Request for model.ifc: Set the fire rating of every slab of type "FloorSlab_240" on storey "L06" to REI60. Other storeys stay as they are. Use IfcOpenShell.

First a look at what the model holds.

```python
import ifcopenshell
import ifcopenshell.util.element

model = ifcopenshell.open("model.ifc")
print(model.schema)
storey = next(s for s in model.by_type("IfcBuildingStorey") if s.Name == "L06")
slabs = [e for e in ifcopenshell.util.element.get_decomposition(storey) if e.is_a("IfcSlab")]
seen = {}
for e in slabs:
    element_type = ifcopenshell.util.element.get_type(e)
    key = (element_type.Name if element_type != e and element_type else None, ifcopenshell.util.element.get_pset(e, "Pset_SlabCommon", "FireRating"))
    seen[key] = seen.get(key, 0) + 1
for (name, value), count in sorted(seen.items(), key=str):
    print(count, "x", name, "|", value)
```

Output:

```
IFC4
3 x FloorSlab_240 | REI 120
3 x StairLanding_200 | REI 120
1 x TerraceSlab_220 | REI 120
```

```python
import ifcopenshell
import ifcopenshell.api.pset
import ifcopenshell.util.element

model = ifcopenshell.open("model.ifc")

storey = next(s for s in model.by_type("IfcBuildingStorey") if s.Name == "L06")
slabs = [e for e in ifcopenshell.util.element.get_decomposition(storey) if e.is_a("IfcSlab")]

count = 0
for e in slabs:
    element_type = ifcopenshell.util.element.get_type(e)
    if element_type in (None, e) or element_type.Name != "FloorSlab_240":
        continue
    # add_pset returns the element's existing set when there is one.
    pset = ifcopenshell.api.pset.add_pset(model, product=e, name="Pset_SlabCommon")
    ifcopenshell.api.pset.edit_pset(model, pset=pset, properties={"FireRating": "REI60"})
    count += 1

print(count, "slabs updated")

model.write("model_edited.ifc")
```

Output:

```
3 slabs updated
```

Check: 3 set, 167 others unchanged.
